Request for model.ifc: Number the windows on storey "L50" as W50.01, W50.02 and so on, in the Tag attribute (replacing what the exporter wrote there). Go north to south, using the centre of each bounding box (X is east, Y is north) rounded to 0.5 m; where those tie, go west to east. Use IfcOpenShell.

First a look at what the model holds.

```python
import ifcopenshell
import ifcopenshell.util.element
import ifcopenshell.util.placement

model = ifcopenshell.open("model.ifc")
print(model.schema)
storey = next(s for s in model.by_type("IfcBuildingStorey") if s.Name == "L50")
windows = [e for e in ifcopenshell.util.element.get_decomposition(storey) if e.is_a("IfcWindow")]
for e in sorted(windows, key=lambda e: e.id()):
    origin = ifcopenshell.util.placement.get_local_placement(e.ObjectPlacement)[:3, 3]
    print(e.id(), e.Tag, e.Name, origin.round(2) + 0.0, sep=" | ")
```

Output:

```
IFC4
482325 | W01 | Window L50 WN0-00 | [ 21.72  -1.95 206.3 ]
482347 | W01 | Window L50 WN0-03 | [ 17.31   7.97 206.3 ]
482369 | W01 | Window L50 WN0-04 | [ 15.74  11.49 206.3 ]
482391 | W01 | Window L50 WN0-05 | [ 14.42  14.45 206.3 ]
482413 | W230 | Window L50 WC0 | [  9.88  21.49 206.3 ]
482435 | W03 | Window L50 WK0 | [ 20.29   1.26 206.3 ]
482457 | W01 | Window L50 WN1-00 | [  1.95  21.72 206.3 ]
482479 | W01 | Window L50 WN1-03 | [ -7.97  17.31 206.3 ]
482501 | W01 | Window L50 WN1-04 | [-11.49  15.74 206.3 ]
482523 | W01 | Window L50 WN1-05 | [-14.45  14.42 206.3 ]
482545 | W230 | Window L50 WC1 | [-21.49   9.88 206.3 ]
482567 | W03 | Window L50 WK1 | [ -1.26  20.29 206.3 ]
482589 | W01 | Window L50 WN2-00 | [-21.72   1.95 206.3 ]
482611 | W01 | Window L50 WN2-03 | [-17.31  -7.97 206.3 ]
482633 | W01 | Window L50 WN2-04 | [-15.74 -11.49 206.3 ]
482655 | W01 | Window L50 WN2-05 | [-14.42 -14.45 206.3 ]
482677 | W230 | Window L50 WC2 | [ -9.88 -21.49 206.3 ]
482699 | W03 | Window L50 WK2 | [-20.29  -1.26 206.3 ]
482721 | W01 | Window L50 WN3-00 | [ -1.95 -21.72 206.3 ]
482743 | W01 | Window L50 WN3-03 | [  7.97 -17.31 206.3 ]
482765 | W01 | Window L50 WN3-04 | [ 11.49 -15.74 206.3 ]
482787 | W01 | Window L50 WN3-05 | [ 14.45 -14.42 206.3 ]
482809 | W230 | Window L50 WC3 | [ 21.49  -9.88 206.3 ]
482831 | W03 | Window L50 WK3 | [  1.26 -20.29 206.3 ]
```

```python
import ifcopenshell
import ifcopenshell.geom
import ifcopenshell.util.element
import ifcopenshell.util.shape

model = ifcopenshell.open("model.ifc")
settings = ifcopenshell.geom.settings()
settings.set("use-world-coords", True)


def centre(element):
    shape = ifcopenshell.geom.create_shape(settings, element)
    return ifcopenshell.util.shape.get_bbox_centroid(shape.geometry)


storey = next(s for s in model.by_type("IfcBuildingStorey") if s.Name == "L50")
windows = [e for e in ifcopenshell.util.element.get_decomposition(storey) if e.is_a("IfcWindow")]

# Insertion points can sit at a corner or the storey origin, so sort by the geometry (in metres).
centres = {e: centre(e) for e in windows}
windows.sort(key=lambda e: (-round(centres[e][1] / 0.5), centres[e][0]))

for i, e in enumerate(windows, start=1):
    number = f"W50.{i:02d}"
    e.Tag = number
    print(e.id(), number)

model.write("model_updated.ifc")
```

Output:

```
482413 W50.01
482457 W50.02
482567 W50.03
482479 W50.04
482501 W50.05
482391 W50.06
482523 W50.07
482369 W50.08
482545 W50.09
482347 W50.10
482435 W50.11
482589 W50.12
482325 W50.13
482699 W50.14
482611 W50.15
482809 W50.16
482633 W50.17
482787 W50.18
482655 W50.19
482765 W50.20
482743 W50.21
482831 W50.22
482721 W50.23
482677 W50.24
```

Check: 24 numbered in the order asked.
